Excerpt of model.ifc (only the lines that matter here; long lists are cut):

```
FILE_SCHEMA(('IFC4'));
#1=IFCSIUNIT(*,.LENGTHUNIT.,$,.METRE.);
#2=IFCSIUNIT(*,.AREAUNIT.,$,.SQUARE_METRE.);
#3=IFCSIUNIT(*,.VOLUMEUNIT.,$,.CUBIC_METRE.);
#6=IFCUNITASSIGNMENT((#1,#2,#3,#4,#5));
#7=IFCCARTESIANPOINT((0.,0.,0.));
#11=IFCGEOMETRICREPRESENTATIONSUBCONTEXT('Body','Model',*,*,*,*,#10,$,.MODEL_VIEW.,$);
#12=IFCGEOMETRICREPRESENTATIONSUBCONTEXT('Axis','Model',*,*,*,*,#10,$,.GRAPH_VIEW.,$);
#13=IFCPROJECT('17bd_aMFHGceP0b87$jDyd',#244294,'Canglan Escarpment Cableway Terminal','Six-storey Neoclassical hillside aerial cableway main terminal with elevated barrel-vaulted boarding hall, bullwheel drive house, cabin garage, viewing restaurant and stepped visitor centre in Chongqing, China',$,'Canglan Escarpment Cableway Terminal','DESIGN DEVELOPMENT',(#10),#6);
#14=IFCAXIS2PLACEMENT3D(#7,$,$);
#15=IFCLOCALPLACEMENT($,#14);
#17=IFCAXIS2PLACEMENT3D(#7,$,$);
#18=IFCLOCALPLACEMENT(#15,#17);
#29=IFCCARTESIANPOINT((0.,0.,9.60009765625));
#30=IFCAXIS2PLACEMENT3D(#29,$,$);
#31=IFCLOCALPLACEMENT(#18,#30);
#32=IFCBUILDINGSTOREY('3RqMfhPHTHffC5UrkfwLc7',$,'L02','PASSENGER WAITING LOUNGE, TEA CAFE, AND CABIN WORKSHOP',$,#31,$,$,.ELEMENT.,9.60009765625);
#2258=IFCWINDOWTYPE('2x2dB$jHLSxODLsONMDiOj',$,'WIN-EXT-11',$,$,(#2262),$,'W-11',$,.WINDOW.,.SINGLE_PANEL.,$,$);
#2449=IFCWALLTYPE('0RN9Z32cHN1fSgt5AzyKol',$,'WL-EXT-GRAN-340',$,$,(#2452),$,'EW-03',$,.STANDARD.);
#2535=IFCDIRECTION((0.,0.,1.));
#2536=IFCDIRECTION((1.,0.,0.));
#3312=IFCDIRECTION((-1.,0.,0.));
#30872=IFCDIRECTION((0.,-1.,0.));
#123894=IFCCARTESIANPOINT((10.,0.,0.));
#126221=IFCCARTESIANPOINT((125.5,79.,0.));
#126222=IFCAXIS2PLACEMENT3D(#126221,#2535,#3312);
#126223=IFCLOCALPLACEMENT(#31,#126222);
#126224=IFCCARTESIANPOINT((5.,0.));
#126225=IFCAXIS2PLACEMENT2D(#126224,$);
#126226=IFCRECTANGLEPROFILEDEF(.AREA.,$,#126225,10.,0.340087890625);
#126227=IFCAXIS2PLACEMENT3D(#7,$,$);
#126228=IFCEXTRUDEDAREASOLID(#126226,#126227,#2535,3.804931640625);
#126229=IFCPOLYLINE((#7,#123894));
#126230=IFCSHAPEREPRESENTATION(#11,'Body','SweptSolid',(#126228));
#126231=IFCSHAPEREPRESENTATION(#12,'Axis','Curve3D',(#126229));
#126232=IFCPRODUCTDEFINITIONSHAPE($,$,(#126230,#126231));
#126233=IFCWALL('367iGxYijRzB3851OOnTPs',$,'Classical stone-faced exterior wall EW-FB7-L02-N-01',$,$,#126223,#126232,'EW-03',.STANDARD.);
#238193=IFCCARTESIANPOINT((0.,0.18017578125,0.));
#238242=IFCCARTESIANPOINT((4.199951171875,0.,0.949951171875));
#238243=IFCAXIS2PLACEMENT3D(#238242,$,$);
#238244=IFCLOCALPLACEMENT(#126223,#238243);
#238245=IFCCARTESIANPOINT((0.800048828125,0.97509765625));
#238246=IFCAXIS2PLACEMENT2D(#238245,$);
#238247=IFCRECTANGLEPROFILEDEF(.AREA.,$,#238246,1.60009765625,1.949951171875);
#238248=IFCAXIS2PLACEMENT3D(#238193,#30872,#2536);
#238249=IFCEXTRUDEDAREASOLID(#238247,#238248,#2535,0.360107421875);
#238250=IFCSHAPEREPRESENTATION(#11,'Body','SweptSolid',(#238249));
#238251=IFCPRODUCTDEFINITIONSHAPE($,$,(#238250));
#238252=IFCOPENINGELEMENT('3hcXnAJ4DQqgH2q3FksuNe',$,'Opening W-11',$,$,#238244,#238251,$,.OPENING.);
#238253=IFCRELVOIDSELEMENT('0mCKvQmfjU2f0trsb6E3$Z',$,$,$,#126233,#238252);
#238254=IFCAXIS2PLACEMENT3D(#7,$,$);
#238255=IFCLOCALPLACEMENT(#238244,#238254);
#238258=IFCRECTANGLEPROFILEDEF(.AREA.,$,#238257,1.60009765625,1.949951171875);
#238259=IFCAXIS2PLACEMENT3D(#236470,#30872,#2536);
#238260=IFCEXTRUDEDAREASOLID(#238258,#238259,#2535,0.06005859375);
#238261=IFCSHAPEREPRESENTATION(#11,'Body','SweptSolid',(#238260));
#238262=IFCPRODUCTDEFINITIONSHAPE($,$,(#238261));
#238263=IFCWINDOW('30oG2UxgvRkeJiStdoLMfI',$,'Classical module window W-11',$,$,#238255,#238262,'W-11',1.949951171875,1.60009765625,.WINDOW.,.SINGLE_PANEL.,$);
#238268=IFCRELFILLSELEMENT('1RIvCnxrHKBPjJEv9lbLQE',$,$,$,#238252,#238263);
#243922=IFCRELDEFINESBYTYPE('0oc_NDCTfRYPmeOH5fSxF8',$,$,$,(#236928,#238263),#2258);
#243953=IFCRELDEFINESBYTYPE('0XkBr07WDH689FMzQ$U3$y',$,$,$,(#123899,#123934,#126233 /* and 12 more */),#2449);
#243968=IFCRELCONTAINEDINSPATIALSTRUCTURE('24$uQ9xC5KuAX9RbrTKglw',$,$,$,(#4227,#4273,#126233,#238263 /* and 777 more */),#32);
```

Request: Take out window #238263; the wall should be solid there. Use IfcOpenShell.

```python
import ifcopenshell
import ifcopenshell.api.feature
import ifcopenshell.api.root
import ifcopenshell.geom
import ifcopenshell.util.shape

model = ifcopenshell.open("model.ifc")
settings = ifcopenshell.geom.settings()


def volume(element):
    """Net volume in cubic metres, openings subtracted."""
    shape = ifcopenshell.geom.create_shape(settings, element)
    return ifcopenshell.util.shape.get_volume(shape.geometry)


window = model.by_id(238263)
opening = window.FillsVoids[0].RelatingOpeningElement
wall = opening.VoidsElements[0].RelatingBuildingElement
before = volume(wall)

ifcopenshell.api.root.remove_product(model, product=window)
ifcopenshell.api.feature.remove_feature(model, feature=opening)

after = volume(wall)

print(f"wall volume {before:.3f} -> {after:.3f} m3")

model.write("model_rev.ifc")
```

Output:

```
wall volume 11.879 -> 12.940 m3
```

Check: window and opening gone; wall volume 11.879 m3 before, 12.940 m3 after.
